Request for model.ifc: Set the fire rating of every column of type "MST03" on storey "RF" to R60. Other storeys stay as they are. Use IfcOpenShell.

First a look at what the model holds.

```python
import ifcopenshell
import ifcopenshell.util.element

model = ifcopenshell.open("model.ifc")
print(model.schema)
storey = next(s for s in model.by_type("IfcBuildingStorey") if s.Name == "RF")
columns = [e for e in ifcopenshell.util.element.get_decomposition(storey) if e.is_a("IfcColumn")]
seen = {}
for e in columns:
    element_type = ifcopenshell.util.element.get_type(e)
    key = (element_type.Name if element_type != e and element_type else None, ifcopenshell.util.element.get_pset(e, "Pset_ColumnCommon", "FireRating"))
    seen[key] = seen.get(key, 0) + 1
for (name, value), count in sorted(seen.items(), key=str):
    print(count, "x", name, "|", value)
```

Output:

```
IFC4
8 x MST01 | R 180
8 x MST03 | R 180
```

```python
import ifcopenshell
import ifcopenshell.api.pset
import ifcopenshell.util.element

model = ifcopenshell.open("model.ifc")

storey = next(s for s in model.by_type("IfcBuildingStorey") if s.Name == "RF")
columns = [e for e in ifcopenshell.util.element.get_decomposition(storey) if e.is_a("IfcColumn")]

count = 0
for e in columns:
    element_type = ifcopenshell.util.element.get_type(e)
    if element_type in (None, e) or element_type.Name != "MST03":
        continue
    # add_pset returns the element's existing set when there is one.
    pset = ifcopenshell.api.pset.add_pset(model, product=e, name="Pset_ColumnCommon")
    ifcopenshell.api.pset.edit_pset(model, pset=pset, properties={"FireRating": "R60"})
    count += 1

print(count, "columns updated")

model.write("model_rev.ifc")
```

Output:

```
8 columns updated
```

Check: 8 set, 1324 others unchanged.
